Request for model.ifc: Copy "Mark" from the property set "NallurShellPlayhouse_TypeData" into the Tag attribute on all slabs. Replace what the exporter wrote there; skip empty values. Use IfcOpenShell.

First a look at what the model holds.

```python
import ifcopenshell
import ifcopenshell.util.element

model = ifcopenshell.open("model.ifc")
print(model.schema)
slabs = model.by_type("IfcSlab")
print(len(slabs), "slabs")
for e in slabs[:8]:
    source = ifcopenshell.util.element.get_pset(e, "NallurShellPlayhouse_TypeData", "Mark")
    target = e.Tag
    print(e.id(), repr(source), repr(target), sep=" | ")
```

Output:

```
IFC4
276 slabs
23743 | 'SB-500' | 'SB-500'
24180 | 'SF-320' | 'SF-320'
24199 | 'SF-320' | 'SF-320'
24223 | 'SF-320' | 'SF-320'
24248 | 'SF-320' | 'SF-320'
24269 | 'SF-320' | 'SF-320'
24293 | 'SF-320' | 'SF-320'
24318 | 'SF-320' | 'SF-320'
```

```python
import ifcopenshell
import ifcopenshell.util.element

model = ifcopenshell.open("model.ifc")

count = 0
for e in model.by_type("IfcSlab"):
    value = ifcopenshell.util.element.get_pset(e, "NallurShellPlayhouse_TypeData", "Mark")
    current = e.Tag
    if not value or not value.strip() or current == value:
        continue
    e.Tag = value
    count += 1

print(count, "slabs updated")

model.write("model_rev.ifc")
```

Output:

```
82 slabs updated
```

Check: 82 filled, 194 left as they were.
